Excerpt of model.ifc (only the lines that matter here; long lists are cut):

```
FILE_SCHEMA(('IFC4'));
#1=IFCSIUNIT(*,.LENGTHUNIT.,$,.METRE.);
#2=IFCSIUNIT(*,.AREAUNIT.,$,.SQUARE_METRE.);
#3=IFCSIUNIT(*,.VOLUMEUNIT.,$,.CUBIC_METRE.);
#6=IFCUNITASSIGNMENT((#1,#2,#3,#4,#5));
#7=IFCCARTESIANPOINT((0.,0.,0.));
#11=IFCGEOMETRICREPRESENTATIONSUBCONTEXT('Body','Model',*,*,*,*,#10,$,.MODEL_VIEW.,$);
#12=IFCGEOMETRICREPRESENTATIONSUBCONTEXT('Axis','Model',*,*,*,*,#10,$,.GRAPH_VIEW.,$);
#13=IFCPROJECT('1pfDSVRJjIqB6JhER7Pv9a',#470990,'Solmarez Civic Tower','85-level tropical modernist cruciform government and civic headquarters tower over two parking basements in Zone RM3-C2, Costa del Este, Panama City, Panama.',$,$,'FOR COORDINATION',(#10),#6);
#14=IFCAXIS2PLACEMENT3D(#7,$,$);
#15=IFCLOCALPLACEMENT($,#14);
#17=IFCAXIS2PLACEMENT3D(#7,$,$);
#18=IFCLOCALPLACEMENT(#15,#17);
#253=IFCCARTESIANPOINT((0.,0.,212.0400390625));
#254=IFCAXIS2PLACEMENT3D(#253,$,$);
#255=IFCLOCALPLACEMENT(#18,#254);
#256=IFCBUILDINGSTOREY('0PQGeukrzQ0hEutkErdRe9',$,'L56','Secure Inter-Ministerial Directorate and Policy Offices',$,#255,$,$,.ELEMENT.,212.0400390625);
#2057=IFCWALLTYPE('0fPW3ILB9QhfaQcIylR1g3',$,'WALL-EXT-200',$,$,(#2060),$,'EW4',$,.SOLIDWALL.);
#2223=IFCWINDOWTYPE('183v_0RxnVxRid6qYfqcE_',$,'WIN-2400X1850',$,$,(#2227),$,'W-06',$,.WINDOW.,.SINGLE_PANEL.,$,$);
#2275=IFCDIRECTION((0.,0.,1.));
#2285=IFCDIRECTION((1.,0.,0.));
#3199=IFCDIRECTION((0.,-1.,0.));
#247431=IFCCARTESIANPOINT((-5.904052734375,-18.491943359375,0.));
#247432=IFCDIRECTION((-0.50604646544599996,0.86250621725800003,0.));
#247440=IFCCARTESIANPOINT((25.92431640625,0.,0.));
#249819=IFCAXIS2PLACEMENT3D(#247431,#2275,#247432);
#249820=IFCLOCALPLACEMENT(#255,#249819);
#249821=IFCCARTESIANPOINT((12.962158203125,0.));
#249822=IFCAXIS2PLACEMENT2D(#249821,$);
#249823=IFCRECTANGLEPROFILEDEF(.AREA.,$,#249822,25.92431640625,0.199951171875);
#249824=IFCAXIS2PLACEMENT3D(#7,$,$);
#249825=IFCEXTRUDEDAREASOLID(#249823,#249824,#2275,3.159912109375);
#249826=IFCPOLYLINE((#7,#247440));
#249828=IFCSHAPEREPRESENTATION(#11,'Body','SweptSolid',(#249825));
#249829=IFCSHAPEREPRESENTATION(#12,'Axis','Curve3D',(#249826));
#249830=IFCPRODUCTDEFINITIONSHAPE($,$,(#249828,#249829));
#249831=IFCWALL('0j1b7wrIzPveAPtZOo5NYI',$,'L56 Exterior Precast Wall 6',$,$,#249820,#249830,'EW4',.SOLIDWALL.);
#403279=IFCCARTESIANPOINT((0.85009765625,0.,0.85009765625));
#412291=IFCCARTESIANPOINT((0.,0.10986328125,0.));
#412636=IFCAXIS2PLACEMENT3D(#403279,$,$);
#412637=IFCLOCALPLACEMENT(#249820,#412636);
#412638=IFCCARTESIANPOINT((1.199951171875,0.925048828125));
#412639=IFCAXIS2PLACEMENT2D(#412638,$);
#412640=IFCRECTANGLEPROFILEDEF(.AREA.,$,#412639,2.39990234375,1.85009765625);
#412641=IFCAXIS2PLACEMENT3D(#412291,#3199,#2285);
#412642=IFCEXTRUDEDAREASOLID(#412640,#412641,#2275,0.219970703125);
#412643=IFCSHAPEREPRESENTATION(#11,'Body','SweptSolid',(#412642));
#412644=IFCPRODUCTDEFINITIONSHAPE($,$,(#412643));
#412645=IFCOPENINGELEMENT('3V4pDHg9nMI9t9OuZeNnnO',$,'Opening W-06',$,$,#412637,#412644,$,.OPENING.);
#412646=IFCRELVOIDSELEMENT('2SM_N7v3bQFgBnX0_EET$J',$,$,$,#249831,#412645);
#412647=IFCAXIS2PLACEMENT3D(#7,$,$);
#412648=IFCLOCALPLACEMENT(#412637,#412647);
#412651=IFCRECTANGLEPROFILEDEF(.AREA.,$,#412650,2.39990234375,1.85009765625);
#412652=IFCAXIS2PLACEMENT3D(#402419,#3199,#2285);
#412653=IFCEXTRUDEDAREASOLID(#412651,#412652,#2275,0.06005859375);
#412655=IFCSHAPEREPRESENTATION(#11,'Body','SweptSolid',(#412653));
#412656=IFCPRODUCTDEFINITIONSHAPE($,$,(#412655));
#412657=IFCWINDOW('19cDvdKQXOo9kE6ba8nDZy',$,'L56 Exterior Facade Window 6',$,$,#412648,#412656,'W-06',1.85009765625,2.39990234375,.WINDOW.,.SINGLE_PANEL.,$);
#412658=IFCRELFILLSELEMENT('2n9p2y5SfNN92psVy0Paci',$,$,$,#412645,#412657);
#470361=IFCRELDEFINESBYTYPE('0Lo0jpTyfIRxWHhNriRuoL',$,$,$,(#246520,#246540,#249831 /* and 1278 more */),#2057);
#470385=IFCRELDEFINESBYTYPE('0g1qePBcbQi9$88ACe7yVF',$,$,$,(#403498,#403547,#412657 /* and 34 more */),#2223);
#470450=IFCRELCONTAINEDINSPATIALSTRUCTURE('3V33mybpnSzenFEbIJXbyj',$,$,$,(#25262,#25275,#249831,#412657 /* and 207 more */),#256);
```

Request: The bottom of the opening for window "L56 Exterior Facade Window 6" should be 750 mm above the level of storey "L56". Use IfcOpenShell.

```python
import numpy as np
import ifcopenshell
import ifcopenshell.api.geometry
import ifcopenshell.geom
import ifcopenshell.util.element
import ifcopenshell.util.placement
import ifcopenshell.util.shape
import ifcopenshell.util.unit

model = ifcopenshell.open("model.ifc")
unit_scale = ifcopenshell.util.unit.calculate_unit_scale(model)

window = model.by_guid("19cDvdKQXOo9kE6ba8nDZy")
opening = window.FillsVoids[0].RelatingOpeningElement
storey = ifcopenshell.util.element.get_container(window, ifc_class="IfcBuildingStorey")
level = ifcopenshell.util.placement.get_local_placement(storey.ObjectPlacement)[2, 3]

# The opening's origin need not be at the sill, so measure its lowest point.
shape = ifcopenshell.geom.create_shape(ifcopenshell.geom.settings(), opening)
bottom = ifcopenshell.util.shape.get_shape_bottom_elevation(shape, shape.geometry) / unit_scale
dz = level + 0.75 / unit_scale - bottom

shift = np.array([0.0, 0.0, dz])
# The window is placed relative to its opening, so it follows when the opening moves.
matrix = ifcopenshell.util.placement.get_local_placement(opening.ObjectPlacement)
matrix[:3, 3] += shift
ifcopenshell.api.geometry.edit_object_placement(
    model, product=opening, matrix=matrix, is_si=False, should_transform_children=True
)

print(f"moved by {dz * unit_scale:+.3f} m")

model.write("model_edited.ifc")
```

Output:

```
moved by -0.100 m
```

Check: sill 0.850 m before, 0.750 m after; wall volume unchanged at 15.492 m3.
